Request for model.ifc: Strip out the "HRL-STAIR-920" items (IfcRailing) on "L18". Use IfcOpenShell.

First a look at what the model holds.

```python
import ifcopenshell
import ifcopenshell.util.element

model = ifcopenshell.open("model.ifc")
print(model.schema)
storey = next(s for s in model.by_type("IfcBuildingStorey") if s.Name == "L18")
railings = [e for e in ifcopenshell.util.element.get_decomposition(storey) if e.is_a("IfcRailing")]
seen = {}
for e in railings:
    element_type = ifcopenshell.util.element.get_type(e)
    name = element_type.Name if element_type not in (None, e) else None
    seen[name] = seen.get(name, 0) + 1
for name, count in sorted(seen.items(), key=str):
    print(count, "x", name)
```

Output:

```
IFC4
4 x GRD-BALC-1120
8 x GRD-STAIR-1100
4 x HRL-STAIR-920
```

```python
import ifcopenshell
import ifcopenshell.api.root
import ifcopenshell.util.element

model = ifcopenshell.open("model.ifc")

storey = next(s for s in model.by_type("IfcBuildingStorey") if s.Name == "L18")
railings = [e for e in ifcopenshell.util.element.get_decomposition(storey) if e.is_a("IfcRailing")]
targets = [e for e in railings if (t := ifcopenshell.util.element.get_type(e)) not in (None, e) and t.Name == "HRL-STAIR-920"]

for e in targets:
    ifcopenshell.api.root.remove_product(model, product=e)
print(len(targets), "removed")

model.write("model_v2.ifc")
```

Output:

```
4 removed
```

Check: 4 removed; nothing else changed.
